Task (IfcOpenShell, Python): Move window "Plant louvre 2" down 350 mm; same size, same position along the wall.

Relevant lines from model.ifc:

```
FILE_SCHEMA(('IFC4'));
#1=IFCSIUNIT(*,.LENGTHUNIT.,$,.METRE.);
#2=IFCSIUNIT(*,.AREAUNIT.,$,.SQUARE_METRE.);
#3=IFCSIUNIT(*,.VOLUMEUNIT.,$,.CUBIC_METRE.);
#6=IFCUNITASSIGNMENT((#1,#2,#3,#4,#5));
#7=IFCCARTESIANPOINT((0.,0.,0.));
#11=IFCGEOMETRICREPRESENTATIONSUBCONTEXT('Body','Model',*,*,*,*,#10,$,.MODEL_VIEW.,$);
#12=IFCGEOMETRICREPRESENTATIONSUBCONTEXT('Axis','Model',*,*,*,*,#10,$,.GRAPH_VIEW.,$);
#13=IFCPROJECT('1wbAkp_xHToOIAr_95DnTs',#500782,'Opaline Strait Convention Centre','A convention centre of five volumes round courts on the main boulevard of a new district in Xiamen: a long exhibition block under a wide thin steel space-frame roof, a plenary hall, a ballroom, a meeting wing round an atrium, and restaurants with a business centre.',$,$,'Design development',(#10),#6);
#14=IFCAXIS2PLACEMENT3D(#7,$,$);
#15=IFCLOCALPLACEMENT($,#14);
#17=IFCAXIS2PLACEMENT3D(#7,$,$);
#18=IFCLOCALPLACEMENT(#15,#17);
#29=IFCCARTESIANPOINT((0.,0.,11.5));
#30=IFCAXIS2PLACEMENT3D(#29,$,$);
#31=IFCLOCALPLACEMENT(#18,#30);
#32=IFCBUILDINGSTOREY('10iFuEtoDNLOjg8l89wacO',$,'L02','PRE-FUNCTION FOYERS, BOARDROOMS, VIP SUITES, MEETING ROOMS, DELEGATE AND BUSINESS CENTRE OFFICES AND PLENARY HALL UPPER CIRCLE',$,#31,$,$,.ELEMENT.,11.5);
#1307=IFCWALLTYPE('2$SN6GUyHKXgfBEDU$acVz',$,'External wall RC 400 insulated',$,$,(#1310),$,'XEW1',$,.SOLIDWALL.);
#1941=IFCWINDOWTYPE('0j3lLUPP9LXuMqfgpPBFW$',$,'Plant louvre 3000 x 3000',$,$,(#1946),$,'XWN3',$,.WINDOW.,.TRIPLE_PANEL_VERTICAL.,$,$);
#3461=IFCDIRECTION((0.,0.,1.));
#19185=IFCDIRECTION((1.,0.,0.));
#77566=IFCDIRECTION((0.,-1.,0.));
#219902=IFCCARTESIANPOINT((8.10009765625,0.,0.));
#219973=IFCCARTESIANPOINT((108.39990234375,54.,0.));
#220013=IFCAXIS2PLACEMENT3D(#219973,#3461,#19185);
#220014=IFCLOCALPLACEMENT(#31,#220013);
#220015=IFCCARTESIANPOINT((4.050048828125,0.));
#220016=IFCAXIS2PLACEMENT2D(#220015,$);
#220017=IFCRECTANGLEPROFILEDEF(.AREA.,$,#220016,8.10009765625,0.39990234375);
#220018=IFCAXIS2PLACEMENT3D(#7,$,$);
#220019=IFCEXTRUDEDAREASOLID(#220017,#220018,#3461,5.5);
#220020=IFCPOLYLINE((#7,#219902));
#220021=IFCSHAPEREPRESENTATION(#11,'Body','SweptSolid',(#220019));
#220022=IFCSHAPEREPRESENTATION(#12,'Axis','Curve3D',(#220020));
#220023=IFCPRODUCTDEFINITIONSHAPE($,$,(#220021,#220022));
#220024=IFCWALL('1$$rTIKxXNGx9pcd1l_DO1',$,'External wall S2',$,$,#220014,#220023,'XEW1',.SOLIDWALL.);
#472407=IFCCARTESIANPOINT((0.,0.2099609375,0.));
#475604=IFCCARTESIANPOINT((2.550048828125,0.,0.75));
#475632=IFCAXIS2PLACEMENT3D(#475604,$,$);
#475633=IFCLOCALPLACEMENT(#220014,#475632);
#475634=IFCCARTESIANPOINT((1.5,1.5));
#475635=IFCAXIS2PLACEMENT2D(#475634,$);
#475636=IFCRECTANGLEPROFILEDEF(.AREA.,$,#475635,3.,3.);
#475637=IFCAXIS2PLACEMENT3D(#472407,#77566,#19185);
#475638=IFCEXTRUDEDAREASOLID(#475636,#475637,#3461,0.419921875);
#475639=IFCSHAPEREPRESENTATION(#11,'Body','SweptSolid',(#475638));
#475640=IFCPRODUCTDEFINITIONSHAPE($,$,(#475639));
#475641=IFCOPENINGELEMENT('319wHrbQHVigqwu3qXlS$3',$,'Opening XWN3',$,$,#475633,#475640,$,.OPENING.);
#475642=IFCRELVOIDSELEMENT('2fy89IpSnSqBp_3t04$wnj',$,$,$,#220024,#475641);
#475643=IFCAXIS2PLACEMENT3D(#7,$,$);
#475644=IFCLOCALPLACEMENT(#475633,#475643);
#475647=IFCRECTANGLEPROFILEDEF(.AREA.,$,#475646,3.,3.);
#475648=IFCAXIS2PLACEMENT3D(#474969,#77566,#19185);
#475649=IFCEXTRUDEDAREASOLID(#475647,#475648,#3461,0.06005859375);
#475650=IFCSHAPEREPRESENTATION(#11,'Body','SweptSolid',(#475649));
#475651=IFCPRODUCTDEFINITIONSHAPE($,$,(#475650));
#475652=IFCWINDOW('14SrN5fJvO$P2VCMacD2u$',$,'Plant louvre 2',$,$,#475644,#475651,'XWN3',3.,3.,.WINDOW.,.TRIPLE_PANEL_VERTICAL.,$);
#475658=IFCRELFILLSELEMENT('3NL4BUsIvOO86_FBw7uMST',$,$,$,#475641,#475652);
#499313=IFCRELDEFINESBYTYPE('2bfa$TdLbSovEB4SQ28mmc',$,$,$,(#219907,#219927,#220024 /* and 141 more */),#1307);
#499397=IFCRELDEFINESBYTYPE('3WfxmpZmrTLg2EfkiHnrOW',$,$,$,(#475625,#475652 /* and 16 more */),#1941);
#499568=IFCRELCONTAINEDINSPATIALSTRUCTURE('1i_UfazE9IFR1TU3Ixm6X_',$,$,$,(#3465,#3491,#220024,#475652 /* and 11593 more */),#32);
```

```python
import numpy as np
import ifcopenshell
import ifcopenshell.api.geometry
import ifcopenshell.util.placement
import ifcopenshell.util.unit

model = ifcopenshell.open("model.ifc")
unit_scale = ifcopenshell.util.unit.calculate_unit_scale(model)

window = model.by_guid("14SrN5fJvO$P2VCMacD2u$")
opening = window.FillsVoids[0].RelatingOpeningElement
dz = -0.35 / unit_scale

shift = np.array([0.0, 0.0, dz])
# The window is placed relative to its opening, so it follows when the opening moves.
matrix = ifcopenshell.util.placement.get_local_placement(opening.ObjectPlacement)
matrix[:3, 3] += shift
ifcopenshell.api.geometry.edit_object_placement(
    model, product=opening, matrix=matrix, is_si=False, should_transform_children=True
)

print(f"moved by {dz * unit_scale:+.3f} m")

model.write("model_v2.ifc")
```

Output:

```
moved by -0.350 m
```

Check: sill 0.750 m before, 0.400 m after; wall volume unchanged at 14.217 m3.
